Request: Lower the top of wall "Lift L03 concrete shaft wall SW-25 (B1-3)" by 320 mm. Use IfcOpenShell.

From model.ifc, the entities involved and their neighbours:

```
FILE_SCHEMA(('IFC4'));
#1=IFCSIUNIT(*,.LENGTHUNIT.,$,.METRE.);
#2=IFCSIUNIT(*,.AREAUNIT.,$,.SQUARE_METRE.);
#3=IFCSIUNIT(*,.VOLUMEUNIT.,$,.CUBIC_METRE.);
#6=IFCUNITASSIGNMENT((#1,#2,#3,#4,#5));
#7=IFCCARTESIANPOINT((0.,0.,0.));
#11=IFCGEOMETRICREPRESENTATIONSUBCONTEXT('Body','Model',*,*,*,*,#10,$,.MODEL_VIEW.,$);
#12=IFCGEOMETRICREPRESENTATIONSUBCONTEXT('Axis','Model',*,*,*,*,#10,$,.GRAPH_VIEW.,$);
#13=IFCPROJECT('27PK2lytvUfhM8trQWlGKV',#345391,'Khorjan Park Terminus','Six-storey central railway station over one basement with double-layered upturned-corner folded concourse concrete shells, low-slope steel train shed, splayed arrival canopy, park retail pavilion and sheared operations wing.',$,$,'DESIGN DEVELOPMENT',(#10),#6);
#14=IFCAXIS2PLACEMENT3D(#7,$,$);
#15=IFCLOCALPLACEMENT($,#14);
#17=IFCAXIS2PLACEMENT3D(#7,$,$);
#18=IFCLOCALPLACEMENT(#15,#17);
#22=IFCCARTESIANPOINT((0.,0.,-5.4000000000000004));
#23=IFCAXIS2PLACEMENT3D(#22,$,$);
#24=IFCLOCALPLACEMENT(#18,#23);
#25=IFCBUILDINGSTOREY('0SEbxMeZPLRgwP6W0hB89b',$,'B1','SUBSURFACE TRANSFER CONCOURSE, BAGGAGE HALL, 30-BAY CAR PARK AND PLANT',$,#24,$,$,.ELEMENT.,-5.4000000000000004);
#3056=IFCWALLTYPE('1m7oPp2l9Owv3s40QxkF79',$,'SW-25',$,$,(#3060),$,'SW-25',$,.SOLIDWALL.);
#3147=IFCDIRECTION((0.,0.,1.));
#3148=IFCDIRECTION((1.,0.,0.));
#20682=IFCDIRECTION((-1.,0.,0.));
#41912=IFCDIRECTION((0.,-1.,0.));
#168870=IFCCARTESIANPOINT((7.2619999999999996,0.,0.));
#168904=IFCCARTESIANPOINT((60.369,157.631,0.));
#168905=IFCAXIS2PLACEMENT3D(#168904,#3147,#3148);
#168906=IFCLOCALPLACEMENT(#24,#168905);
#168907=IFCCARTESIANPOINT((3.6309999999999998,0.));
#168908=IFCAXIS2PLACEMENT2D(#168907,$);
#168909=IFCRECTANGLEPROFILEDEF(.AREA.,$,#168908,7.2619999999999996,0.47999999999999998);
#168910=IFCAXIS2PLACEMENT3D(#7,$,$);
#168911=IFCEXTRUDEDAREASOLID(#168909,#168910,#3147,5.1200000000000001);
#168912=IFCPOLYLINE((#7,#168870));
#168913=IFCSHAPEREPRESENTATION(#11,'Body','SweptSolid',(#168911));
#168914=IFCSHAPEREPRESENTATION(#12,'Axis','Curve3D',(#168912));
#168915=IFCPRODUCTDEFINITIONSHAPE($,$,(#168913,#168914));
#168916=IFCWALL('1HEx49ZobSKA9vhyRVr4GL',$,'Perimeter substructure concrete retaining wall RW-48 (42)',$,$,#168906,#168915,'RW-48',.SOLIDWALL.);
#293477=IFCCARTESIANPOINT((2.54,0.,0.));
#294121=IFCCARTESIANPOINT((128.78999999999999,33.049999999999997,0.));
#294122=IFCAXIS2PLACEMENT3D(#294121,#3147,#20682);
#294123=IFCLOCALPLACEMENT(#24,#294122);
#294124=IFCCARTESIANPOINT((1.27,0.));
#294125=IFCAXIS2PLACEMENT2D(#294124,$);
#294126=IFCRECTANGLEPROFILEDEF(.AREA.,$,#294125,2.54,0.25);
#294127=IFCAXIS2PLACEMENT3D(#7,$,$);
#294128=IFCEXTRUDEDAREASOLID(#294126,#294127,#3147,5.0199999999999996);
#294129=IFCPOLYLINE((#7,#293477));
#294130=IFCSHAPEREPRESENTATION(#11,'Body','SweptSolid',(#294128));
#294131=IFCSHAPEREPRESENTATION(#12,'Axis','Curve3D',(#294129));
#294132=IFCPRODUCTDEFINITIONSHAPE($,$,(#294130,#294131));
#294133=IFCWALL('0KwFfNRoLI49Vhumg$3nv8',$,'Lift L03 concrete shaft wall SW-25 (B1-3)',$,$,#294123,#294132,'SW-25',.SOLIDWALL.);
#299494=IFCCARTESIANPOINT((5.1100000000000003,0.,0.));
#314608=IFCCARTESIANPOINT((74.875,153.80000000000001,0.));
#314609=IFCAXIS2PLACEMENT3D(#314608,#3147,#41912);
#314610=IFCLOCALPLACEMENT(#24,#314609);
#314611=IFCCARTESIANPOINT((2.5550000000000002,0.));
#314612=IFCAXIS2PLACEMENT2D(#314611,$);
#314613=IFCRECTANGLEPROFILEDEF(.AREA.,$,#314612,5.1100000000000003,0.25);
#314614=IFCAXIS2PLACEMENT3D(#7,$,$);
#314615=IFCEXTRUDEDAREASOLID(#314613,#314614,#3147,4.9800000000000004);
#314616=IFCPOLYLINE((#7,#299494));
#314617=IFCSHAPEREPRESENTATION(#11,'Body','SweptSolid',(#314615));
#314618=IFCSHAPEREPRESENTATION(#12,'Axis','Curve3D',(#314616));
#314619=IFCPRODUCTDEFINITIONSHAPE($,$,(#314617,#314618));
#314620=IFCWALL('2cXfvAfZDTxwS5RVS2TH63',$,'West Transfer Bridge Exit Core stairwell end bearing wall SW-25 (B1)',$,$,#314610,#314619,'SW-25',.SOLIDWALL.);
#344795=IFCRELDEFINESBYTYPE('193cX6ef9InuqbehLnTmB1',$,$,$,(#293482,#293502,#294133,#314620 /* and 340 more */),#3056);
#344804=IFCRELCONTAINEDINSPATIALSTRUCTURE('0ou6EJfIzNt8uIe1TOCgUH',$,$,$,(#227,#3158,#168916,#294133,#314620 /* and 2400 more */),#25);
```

```python
import ifcopenshell
import ifcopenshell.geom
import ifcopenshell.util.representation
import ifcopenshell.util.shape
import ifcopenshell.util.unit

model = ifcopenshell.open("model.ifc")
unit_scale = ifcopenshell.util.unit.calculate_unit_scale(model)
settings = ifcopenshell.geom.settings()


def volume(element):
    """Net volume in cubic metres, openings subtracted."""
    shape = ifcopenshell.geom.create_shape(settings, element)
    return ifcopenshell.util.shape.get_volume(shape.geometry)


wall = model.by_guid("0KwFfNRoLI49Vhumg$3nv8")
before = volume(wall)

body = ifcopenshell.util.representation.get_representation(wall, "Model", "Body")
solid = body.Items[0]
old_height = solid.Depth
solid.Depth -= 0.32 / unit_scale
after = volume(wall)

print(f"height {old_height:g} -> {solid.Depth:g}, volume {before:.3f} -> {after:.3f} m3")

model.write("model_updated.ifc")
```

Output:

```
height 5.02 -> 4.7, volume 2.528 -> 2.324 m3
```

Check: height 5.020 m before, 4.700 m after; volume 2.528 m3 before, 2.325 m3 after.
